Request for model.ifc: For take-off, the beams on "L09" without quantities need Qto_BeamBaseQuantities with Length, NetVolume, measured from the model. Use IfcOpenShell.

First a look at what the model holds.

```python
import ifcopenshell
import ifcopenshell.util.element
import ifcopenshell.util.unit

model = ifcopenshell.open("model.ifc")
print(model.schema)
for unit_type in ("LENGTHUNIT", "AREAUNIT", "VOLUMEUNIT"):
    print(unit_type, ifcopenshell.util.unit.calculate_unit_scale(model, unit_type))
storey = next(s for s in model.by_type("IfcBuildingStorey") if s.Name == "L09")
beams = [e for e in ifcopenshell.util.element.get_decomposition(storey) if e.is_a("IfcBeam")]
for e in sorted(beams, key=lambda e: e.id()):
    print(e.id(), e.is_a(), e.Name, list(ifcopenshell.util.element.get_psets(e, qtos_only=True)), sep=" | ")
```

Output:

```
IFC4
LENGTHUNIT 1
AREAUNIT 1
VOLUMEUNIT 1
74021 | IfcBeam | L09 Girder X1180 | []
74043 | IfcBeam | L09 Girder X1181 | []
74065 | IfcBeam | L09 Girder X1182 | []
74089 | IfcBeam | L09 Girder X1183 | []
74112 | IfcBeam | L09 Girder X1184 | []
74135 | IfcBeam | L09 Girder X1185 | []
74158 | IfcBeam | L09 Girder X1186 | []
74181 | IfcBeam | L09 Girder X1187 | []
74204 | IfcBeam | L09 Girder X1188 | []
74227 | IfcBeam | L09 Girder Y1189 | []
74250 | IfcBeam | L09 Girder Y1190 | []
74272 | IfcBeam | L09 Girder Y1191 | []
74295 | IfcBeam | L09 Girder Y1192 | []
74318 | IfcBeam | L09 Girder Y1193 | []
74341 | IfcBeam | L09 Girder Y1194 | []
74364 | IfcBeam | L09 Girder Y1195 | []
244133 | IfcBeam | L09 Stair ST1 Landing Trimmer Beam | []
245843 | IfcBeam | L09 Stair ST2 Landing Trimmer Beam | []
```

```python
import ifcopenshell
import ifcopenshell.api.pset
import ifcopenshell.geom
import ifcopenshell.util.element
import ifcopenshell.util.shape
import ifcopenshell.util.unit

model = ifcopenshell.open("model.ifc")
unit_scale = ifcopenshell.util.unit.calculate_unit_scale(model)
volume_scale = ifcopenshell.util.unit.calculate_unit_scale(model, "VOLUMEUNIT")
settings = ifcopenshell.geom.settings()

storey = next(s for s in model.by_type("IfcBuildingStorey") if s.Name == "L09")
beams = [e for e in ifcopenshell.util.element.get_decomposition(storey) if e.is_a("IfcBeam")]

for e in sorted(beams, key=lambda e: e.id()):
    if ifcopenshell.util.element.get_psets(e, qtos_only=True, should_inherit=False):
        continue
    # Geometry comes back in metres, in the element's own axes.
    shape = ifcopenshell.geom.create_shape(settings, e)
    values = {
        "Length": ifcopenshell.util.shape.get_max_xyz(shape.geometry) / unit_scale,
        "NetVolume": ifcopenshell.util.shape.get_volume(shape.geometry) / volume_scale,
    }
    qto = ifcopenshell.api.pset.add_qto(model, product=e, name="Qto_BeamBaseQuantities")
    ifcopenshell.api.pset.edit_qto(model, qto=qto, properties=values)
    print(e.id(), {k: round(v, 3) for k, v in values.items()})

model.write("model_updated.ifc")
```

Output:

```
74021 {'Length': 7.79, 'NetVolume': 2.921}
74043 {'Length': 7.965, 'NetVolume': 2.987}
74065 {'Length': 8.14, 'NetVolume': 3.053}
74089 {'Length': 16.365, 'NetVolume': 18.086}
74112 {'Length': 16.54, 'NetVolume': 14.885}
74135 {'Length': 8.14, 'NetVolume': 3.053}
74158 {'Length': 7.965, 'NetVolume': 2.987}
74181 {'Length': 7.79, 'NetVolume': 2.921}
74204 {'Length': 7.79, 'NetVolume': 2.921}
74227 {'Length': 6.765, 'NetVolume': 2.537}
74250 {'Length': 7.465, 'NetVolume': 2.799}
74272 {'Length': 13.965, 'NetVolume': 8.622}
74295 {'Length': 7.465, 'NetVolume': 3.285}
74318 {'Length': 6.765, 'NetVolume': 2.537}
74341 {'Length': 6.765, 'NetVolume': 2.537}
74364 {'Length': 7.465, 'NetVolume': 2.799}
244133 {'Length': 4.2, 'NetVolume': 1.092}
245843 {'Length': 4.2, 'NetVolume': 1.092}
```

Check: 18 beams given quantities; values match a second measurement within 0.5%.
